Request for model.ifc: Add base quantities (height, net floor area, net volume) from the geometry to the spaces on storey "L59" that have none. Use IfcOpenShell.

First a look at what the model holds.

```python
import ifcopenshell
import ifcopenshell.util.element
import ifcopenshell.util.unit

model = ifcopenshell.open("model.ifc")
print(model.schema)
for unit_type in ("LENGTHUNIT", "AREAUNIT", "VOLUMEUNIT"):
    print(unit_type, ifcopenshell.util.unit.calculate_unit_scale(model, unit_type))
storey = next(s for s in model.by_type("IfcBuildingStorey") if s.Name == "L59")
spaces = [e for e in ifcopenshell.util.element.get_decomposition(storey) if e.is_a("IfcSpace")]
for e in sorted(spaces, key=lambda e: e.id()):
    print(e.id(), e.is_a(), e.Name, list(ifcopenshell.util.element.get_psets(e, qtos_only=True)), sep=" | ")
```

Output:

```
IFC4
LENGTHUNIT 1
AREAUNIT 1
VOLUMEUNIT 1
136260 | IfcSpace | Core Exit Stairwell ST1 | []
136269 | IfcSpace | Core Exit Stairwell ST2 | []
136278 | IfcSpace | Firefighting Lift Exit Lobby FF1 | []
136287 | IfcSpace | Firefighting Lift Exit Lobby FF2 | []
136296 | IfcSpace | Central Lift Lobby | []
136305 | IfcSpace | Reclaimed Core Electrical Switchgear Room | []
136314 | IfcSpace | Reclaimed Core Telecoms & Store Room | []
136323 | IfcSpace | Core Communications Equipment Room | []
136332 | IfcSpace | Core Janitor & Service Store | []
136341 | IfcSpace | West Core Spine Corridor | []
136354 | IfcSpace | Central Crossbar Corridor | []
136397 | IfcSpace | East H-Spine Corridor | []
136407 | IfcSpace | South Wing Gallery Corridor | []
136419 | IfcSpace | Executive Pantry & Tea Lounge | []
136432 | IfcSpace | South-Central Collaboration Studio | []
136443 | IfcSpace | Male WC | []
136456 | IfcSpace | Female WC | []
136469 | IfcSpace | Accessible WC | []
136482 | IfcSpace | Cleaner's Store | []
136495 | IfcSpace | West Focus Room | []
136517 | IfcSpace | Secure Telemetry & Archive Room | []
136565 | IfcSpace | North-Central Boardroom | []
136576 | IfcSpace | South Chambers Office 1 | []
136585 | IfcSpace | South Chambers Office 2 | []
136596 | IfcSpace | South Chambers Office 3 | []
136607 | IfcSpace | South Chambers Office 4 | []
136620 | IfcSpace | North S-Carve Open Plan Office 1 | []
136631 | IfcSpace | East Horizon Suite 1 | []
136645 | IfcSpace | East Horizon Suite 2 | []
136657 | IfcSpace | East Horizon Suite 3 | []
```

```python
import ifcopenshell
import ifcopenshell.api.pset
import ifcopenshell.geom
import ifcopenshell.util.element
import ifcopenshell.util.shape
import ifcopenshell.util.unit

model = ifcopenshell.open("model.ifc")
unit_scale = ifcopenshell.util.unit.calculate_unit_scale(model)
area_scale = ifcopenshell.util.unit.calculate_unit_scale(model, "AREAUNIT")
volume_scale = ifcopenshell.util.unit.calculate_unit_scale(model, "VOLUMEUNIT")
settings = ifcopenshell.geom.settings()

storey = next(s for s in model.by_type("IfcBuildingStorey") if s.Name == "L59")
spaces = [e for e in ifcopenshell.util.element.get_decomposition(storey) if e.is_a("IfcSpace")]

for e in sorted(spaces, key=lambda e: e.id()):
    if ifcopenshell.util.element.get_psets(e, qtos_only=True, should_inherit=False):
        continue
    # Geometry comes back in metres, in the element's own axes.
    shape = ifcopenshell.geom.create_shape(settings, e)
    values = {
        "Height": ifcopenshell.util.shape.get_z(shape.geometry) / unit_scale,
        "NetFloorArea": ifcopenshell.util.shape.get_footprint_area(shape.geometry) / area_scale,
        "NetVolume": ifcopenshell.util.shape.get_volume(shape.geometry) / volume_scale,
    }
    qto = ifcopenshell.api.pset.add_qto(model, product=e, name="Qto_SpaceBaseQuantities")
    ifcopenshell.api.pset.edit_qto(model, qto=qto, properties=values)
    print(e.id(), {k: round(v, 3) for k, v in values.items()})

model.write("model-out.ifc")
```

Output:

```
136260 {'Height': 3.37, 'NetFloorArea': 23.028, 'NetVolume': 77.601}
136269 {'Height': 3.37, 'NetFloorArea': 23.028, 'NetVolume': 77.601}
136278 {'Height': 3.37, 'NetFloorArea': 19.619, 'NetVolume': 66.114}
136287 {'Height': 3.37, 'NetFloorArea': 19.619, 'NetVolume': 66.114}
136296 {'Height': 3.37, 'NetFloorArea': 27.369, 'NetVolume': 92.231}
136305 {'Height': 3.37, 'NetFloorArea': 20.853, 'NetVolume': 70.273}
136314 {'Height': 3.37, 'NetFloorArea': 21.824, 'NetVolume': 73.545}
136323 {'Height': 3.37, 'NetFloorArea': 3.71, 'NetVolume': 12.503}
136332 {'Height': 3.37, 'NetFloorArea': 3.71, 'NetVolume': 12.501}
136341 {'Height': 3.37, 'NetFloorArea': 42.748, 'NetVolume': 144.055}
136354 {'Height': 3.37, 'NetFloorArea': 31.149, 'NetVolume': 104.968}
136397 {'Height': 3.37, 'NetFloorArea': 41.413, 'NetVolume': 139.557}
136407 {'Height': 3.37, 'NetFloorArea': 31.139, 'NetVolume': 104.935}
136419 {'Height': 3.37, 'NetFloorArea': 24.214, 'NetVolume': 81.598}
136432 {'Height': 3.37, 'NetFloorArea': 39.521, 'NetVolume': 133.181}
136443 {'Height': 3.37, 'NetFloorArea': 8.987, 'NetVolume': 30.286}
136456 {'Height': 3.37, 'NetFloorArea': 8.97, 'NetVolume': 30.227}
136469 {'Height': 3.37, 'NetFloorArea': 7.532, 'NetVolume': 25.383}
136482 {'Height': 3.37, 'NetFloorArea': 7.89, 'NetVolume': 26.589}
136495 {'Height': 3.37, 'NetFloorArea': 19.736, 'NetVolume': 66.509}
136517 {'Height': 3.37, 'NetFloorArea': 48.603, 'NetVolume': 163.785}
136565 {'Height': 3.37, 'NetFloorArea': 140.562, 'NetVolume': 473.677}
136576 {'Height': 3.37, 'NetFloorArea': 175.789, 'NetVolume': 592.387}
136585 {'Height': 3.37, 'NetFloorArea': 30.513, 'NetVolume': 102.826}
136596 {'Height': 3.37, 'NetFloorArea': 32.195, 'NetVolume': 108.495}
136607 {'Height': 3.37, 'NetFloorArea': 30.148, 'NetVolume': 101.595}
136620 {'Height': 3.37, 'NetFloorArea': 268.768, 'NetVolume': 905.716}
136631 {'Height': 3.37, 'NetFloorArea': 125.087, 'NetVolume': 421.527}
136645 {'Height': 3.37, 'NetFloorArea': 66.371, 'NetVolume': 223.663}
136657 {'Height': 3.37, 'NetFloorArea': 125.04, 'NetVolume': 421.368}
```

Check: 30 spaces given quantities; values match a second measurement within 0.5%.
